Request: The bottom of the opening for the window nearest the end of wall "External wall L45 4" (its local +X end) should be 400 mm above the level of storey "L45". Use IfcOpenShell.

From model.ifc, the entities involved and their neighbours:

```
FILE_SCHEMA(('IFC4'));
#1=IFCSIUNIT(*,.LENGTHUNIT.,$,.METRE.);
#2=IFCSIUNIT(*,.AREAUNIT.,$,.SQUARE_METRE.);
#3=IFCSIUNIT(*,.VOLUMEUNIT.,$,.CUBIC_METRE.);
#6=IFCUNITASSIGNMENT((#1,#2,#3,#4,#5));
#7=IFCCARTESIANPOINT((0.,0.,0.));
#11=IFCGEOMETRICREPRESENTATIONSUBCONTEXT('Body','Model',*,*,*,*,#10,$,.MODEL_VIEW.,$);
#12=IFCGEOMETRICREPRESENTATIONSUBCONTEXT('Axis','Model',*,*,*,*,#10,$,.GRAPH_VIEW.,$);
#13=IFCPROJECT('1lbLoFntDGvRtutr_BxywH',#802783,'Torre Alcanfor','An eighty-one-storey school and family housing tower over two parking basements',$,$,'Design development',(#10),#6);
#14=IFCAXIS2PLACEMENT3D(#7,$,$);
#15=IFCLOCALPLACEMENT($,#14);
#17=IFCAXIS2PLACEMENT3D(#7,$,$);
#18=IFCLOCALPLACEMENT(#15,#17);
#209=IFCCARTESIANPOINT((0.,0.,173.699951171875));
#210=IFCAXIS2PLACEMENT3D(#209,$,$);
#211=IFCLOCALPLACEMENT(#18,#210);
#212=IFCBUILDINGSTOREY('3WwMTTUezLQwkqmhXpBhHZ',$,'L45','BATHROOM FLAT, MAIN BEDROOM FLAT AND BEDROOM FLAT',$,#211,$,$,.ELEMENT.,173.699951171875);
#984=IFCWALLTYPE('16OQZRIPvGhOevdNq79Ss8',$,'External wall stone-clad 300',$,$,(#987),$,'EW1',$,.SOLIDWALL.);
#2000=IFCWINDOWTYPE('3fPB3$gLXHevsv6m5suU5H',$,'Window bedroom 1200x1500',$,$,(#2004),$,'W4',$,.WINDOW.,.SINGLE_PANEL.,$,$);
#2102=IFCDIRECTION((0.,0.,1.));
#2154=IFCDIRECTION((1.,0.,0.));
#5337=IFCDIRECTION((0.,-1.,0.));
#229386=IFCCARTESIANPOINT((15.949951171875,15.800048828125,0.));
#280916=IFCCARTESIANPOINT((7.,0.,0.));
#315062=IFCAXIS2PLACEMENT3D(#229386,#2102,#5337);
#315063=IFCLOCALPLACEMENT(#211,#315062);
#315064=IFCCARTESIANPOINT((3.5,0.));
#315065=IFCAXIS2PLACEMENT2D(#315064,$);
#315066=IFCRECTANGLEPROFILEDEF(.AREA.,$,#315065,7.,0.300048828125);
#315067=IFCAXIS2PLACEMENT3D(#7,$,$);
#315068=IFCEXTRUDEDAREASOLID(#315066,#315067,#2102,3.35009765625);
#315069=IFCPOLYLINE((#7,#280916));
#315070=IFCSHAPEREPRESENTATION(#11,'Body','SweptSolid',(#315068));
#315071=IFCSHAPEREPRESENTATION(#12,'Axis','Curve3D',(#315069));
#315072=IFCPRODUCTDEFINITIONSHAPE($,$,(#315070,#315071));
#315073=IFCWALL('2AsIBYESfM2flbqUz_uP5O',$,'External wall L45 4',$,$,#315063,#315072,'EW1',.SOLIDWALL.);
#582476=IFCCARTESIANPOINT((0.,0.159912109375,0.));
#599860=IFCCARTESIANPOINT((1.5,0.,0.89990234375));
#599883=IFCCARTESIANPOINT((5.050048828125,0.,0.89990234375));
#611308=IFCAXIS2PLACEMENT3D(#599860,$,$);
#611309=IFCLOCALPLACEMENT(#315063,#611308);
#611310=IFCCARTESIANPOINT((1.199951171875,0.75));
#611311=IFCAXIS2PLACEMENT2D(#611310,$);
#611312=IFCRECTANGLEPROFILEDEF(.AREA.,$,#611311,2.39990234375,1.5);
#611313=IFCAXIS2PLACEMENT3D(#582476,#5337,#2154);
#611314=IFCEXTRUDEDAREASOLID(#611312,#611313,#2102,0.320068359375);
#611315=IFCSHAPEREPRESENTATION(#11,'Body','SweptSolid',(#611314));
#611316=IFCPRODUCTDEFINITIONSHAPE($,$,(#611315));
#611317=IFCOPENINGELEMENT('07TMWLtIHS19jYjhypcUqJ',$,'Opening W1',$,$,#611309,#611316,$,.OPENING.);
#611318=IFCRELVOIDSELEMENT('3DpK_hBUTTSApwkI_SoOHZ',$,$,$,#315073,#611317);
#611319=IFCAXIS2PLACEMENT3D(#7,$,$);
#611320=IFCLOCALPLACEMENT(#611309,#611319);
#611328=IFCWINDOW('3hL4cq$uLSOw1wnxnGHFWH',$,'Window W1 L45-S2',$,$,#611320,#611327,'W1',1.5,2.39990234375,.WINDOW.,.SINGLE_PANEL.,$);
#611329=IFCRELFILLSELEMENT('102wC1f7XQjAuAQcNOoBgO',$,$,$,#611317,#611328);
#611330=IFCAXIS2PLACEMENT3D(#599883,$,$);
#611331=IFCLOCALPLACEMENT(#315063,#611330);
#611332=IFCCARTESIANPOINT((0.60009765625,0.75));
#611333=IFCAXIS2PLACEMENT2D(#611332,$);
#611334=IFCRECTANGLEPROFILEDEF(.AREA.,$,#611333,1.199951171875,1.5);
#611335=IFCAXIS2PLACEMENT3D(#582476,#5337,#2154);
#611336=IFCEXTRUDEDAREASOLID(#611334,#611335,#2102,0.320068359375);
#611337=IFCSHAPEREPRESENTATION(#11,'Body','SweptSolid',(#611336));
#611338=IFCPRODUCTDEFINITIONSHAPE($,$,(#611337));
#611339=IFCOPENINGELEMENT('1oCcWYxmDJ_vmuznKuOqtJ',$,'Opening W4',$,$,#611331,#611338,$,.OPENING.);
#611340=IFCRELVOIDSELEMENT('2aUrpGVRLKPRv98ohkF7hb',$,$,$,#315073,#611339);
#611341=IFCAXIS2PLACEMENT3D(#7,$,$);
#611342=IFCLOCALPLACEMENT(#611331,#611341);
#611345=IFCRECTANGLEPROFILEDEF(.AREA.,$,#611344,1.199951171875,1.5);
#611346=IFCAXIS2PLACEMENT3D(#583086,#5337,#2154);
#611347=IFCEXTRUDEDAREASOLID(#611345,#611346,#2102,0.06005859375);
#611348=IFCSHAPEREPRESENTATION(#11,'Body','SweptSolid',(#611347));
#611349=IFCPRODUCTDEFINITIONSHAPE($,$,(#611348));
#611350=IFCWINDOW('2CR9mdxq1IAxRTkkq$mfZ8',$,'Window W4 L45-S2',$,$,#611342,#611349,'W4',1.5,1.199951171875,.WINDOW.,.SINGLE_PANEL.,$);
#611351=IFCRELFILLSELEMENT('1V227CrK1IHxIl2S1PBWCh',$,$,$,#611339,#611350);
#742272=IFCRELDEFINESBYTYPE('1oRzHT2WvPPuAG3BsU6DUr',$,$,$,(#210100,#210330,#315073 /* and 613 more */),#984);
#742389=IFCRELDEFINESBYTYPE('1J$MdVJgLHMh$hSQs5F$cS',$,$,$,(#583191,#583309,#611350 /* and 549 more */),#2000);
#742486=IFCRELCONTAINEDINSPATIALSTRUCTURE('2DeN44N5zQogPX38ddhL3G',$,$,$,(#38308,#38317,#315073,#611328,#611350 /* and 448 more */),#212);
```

```python
import numpy as np
import ifcopenshell
import ifcopenshell.api.geometry
import ifcopenshell.geom
import ifcopenshell.util.element
import ifcopenshell.util.placement
import ifcopenshell.util.shape
import ifcopenshell.util.unit

model = ifcopenshell.open("model.ifc")
unit_scale = ifcopenshell.util.unit.calculate_unit_scale(model)

window = model.by_guid("2CR9mdxq1IAxRTkkq$mfZ8")
opening = window.FillsVoids[0].RelatingOpeningElement
storey = ifcopenshell.util.element.get_container(window, ifc_class="IfcBuildingStorey")
level = ifcopenshell.util.placement.get_local_placement(storey.ObjectPlacement)[2, 3]

# The opening's origin need not be at the sill, so measure its lowest point.
shape = ifcopenshell.geom.create_shape(ifcopenshell.geom.settings(), opening)
bottom = ifcopenshell.util.shape.get_shape_bottom_elevation(shape, shape.geometry) / unit_scale
dz = level + 0.4 / unit_scale - bottom

shift = np.array([0.0, 0.0, dz])
# The window is placed relative to its opening, so it follows when the opening moves.
matrix = ifcopenshell.util.placement.get_local_placement(opening.ObjectPlacement)
matrix[:3, 3] += shift
ifcopenshell.api.geometry.edit_object_placement(
    model, product=opening, matrix=matrix, is_si=False, should_transform_children=True
)

print(f"moved by {dz * unit_scale:+.3f} m")

model.write("model_edited.ifc")
```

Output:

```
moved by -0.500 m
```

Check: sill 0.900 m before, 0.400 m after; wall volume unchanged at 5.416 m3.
